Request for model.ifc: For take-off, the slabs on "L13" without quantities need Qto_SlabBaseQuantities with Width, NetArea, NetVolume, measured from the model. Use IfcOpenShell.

First a look at what the model holds.

```python
import ifcopenshell
import ifcopenshell.util.element
import ifcopenshell.util.unit

model = ifcopenshell.open("model.ifc")
print(model.schema)
for unit_type in ("LENGTHUNIT", "AREAUNIT", "VOLUMEUNIT"):
    print(unit_type, ifcopenshell.util.unit.calculate_unit_scale(model, unit_type))
storey = next(s for s in model.by_type("IfcBuildingStorey") if s.Name == "L13")
slabs = [e for e in ifcopenshell.util.element.get_decomposition(storey) if e.is_a("IfcSlab")]
for e in sorted(slabs, key=lambda e: e.id()):
    print(e.id(), e.is_a(), e.Name, list(ifcopenshell.util.element.get_psets(e, qtos_only=True)), sep=" | ")
```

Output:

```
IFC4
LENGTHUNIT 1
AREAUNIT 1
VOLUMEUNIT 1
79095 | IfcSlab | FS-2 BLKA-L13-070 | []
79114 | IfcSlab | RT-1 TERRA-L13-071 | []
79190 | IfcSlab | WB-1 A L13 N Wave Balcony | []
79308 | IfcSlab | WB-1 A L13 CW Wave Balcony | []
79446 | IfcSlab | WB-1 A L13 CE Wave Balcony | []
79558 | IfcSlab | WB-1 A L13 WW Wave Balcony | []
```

```python
import ifcopenshell
import ifcopenshell.api.pset
import ifcopenshell.geom
import ifcopenshell.util.element
import ifcopenshell.util.shape
import ifcopenshell.util.unit

model = ifcopenshell.open("model.ifc")
unit_scale = ifcopenshell.util.unit.calculate_unit_scale(model)
area_scale = ifcopenshell.util.unit.calculate_unit_scale(model, "AREAUNIT")
volume_scale = ifcopenshell.util.unit.calculate_unit_scale(model, "VOLUMEUNIT")
settings = ifcopenshell.geom.settings()

storey = next(s for s in model.by_type("IfcBuildingStorey") if s.Name == "L13")
slabs = [e for e in ifcopenshell.util.element.get_decomposition(storey) if e.is_a("IfcSlab")]

for e in sorted(slabs, key=lambda e: e.id()):
    if ifcopenshell.util.element.get_psets(e, qtos_only=True, should_inherit=False):
        continue
    # Geometry comes back in metres, in the element's own axes.
    shape = ifcopenshell.geom.create_shape(settings, e)
    values = {
        "Width": ifcopenshell.util.shape.get_z(shape.geometry) / unit_scale,
        "NetArea": ifcopenshell.util.shape.get_footprint_area(shape.geometry) / area_scale,
        "NetVolume": ifcopenshell.util.shape.get_volume(shape.geometry) / volume_scale,
    }
    qto = ifcopenshell.api.pset.add_qto(model, product=e, name="Qto_SlabBaseQuantities")
    ifcopenshell.api.pset.edit_qto(model, qto=qto, properties=values)
    print(e.id(), {k: round(v, 3) for k, v in values.items()})

model.write("model-out.ifc")
```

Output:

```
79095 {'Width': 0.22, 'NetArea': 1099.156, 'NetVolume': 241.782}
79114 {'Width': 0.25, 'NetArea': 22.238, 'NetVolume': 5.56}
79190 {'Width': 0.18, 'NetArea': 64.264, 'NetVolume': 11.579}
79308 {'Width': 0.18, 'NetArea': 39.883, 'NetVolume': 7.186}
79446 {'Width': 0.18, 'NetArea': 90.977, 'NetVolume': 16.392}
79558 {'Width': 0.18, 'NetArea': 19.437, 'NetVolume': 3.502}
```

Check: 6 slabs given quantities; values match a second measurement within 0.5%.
